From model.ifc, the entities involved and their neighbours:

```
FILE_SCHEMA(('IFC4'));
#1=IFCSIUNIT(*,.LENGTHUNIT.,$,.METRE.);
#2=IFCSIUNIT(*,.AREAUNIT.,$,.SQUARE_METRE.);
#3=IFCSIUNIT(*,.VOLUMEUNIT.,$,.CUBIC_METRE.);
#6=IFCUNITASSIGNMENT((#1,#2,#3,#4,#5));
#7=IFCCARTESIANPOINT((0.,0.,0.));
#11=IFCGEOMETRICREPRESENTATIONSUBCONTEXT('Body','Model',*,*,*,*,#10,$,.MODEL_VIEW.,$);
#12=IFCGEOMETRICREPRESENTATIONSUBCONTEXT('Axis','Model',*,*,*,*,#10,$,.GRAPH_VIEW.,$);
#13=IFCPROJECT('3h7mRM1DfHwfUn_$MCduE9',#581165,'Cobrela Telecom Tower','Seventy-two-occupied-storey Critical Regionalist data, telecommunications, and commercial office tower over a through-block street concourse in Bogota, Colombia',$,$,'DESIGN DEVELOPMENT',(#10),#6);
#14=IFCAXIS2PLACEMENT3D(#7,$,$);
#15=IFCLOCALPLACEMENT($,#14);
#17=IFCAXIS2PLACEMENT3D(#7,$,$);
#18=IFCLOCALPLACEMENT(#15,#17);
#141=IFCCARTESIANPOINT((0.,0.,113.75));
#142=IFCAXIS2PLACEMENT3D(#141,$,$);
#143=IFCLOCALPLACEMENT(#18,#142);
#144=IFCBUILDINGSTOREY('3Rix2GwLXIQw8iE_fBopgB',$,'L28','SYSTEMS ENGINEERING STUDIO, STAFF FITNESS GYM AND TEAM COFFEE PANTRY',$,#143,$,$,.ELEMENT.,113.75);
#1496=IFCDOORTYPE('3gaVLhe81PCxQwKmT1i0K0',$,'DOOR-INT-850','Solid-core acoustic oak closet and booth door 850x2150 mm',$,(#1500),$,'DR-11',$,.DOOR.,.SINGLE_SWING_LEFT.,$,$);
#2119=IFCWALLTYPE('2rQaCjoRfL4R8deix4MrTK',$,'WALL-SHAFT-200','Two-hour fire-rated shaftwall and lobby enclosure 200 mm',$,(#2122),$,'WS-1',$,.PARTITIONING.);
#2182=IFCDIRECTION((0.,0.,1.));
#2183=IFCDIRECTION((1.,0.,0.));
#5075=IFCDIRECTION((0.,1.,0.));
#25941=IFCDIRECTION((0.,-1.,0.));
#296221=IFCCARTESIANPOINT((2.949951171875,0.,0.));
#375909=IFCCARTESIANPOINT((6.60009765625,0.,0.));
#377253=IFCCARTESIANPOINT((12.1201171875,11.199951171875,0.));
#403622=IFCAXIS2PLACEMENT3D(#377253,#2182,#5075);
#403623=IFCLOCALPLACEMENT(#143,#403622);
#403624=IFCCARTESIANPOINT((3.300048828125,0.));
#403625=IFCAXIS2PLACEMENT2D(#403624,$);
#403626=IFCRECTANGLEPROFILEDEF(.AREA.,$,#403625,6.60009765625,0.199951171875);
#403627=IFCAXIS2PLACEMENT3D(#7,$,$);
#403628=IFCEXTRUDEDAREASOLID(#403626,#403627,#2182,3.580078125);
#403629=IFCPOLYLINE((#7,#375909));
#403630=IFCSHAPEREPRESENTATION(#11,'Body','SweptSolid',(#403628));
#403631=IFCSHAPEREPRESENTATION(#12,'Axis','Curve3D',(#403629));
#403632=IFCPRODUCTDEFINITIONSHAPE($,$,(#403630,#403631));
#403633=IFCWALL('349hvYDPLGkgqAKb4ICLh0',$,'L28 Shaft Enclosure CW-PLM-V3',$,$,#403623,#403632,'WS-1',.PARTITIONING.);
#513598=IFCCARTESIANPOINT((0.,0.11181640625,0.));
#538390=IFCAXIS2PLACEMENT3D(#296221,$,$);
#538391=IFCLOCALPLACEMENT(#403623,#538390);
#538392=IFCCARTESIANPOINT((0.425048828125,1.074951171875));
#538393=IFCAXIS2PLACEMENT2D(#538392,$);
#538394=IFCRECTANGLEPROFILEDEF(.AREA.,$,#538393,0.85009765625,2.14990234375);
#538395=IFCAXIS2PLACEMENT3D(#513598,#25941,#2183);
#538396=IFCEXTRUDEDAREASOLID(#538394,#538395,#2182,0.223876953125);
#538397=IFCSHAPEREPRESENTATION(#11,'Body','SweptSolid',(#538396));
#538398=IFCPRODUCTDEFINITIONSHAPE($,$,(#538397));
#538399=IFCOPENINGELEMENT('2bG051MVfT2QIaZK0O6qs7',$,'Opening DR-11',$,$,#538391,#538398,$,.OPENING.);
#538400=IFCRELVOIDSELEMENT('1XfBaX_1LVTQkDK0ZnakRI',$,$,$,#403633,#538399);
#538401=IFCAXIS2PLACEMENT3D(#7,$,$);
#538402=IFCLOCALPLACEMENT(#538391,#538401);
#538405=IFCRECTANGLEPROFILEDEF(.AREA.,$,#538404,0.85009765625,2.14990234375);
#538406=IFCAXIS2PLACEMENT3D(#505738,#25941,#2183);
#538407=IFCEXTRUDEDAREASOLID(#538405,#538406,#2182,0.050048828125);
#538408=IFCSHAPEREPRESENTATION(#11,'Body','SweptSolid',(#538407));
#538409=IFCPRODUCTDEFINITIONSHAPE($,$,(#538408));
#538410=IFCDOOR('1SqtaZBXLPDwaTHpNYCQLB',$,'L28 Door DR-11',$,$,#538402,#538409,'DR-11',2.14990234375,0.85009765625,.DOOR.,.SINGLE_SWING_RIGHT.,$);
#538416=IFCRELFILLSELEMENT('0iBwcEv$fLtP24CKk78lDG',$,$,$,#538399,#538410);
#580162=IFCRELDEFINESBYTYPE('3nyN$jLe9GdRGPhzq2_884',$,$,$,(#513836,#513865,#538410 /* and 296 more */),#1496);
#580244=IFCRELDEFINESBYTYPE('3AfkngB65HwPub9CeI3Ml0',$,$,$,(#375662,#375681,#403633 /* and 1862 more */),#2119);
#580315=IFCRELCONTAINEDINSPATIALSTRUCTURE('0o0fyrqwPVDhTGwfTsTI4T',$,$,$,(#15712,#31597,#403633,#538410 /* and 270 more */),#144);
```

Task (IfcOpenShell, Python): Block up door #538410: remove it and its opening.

```python
import ifcopenshell
import ifcopenshell.api.feature
import ifcopenshell.api.root
import ifcopenshell.geom
import ifcopenshell.util.shape

model = ifcopenshell.open("model.ifc")
settings = ifcopenshell.geom.settings()


def volume(element):
    """Net volume in cubic metres, openings subtracted."""
    shape = ifcopenshell.geom.create_shape(settings, element)
    return ifcopenshell.util.shape.get_volume(shape.geometry)


door = model.by_guid("1SqtaZBXLPDwaTHpNYCQLB")
opening = door.FillsVoids[0].RelatingOpeningElement
wall = opening.VoidsElements[0].RelatingBuildingElement
before = volume(wall)

ifcopenshell.api.root.remove_product(model, product=door)
ifcopenshell.api.feature.remove_feature(model, feature=opening)

after = volume(wall)

print(f"wall volume {before:.3f} -> {after:.3f} m3")

model.write("model_updated.ifc")
```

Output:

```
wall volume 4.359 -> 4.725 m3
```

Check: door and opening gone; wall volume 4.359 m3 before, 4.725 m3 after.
